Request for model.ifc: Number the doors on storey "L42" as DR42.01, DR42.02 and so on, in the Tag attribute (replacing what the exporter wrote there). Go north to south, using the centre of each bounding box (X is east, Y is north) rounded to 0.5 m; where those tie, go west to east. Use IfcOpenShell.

First a look at what the model holds.

```python
import ifcopenshell
import ifcopenshell.util.element
import ifcopenshell.util.placement

model = ifcopenshell.open("model.ifc")
print(model.schema)
storey = next(s for s in model.by_type("IfcBuildingStorey") if s.Name == "L42")
doors = [e for e in ifcopenshell.util.element.get_decomposition(storey) if e.is_a("IfcDoor")]
for e in sorted(doors, key=lambda e: e.id()):
    origin = ifcopenshell.util.placement.get_local_placement(e.ObjectPlacement)[:3, 3]
    print(e.id(), e.Tag, e.Name, origin.round(2) + 0.0, sep=" | ")
```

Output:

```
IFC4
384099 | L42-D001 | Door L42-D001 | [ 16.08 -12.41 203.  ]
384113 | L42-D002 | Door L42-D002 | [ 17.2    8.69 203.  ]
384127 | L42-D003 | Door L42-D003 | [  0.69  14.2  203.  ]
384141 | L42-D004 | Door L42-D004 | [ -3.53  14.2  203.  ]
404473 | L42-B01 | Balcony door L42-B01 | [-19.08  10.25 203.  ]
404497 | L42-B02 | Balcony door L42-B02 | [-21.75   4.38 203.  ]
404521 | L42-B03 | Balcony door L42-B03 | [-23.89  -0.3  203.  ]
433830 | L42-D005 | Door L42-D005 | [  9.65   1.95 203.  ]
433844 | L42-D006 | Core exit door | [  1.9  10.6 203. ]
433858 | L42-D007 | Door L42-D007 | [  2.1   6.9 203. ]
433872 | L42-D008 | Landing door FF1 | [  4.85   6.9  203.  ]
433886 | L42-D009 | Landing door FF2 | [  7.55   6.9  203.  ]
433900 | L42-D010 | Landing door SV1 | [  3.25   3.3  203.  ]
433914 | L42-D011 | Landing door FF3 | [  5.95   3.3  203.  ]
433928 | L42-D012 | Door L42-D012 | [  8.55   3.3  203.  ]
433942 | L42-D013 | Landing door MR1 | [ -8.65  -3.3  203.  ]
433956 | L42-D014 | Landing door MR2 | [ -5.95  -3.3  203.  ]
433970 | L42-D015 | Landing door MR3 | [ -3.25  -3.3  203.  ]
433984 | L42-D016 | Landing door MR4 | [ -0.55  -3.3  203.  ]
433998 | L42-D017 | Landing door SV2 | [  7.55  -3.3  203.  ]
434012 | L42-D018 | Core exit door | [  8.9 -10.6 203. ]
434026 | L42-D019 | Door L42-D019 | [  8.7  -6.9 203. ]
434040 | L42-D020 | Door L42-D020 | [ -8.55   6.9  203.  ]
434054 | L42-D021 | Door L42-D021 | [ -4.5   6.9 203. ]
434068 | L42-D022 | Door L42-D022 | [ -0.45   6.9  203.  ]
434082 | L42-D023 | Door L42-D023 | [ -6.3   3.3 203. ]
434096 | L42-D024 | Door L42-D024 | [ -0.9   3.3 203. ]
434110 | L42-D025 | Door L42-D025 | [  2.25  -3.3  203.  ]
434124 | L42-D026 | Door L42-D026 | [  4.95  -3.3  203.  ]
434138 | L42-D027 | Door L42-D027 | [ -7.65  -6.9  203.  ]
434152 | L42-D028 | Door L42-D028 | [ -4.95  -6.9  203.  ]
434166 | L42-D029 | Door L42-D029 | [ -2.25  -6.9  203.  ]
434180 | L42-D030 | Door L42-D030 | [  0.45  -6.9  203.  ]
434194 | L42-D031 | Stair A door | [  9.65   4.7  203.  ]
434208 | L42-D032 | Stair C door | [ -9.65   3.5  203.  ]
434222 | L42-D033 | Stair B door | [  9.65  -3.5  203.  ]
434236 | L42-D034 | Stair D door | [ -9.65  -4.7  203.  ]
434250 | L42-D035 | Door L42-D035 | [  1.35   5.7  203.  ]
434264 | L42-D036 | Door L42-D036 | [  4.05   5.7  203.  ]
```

```python
import ifcopenshell
import ifcopenshell.geom
import ifcopenshell.util.element
import ifcopenshell.util.shape

model = ifcopenshell.open("model.ifc")
settings = ifcopenshell.geom.settings()
settings.set("use-world-coords", True)


def centre(element):
    shape = ifcopenshell.geom.create_shape(settings, element)
    return ifcopenshell.util.shape.get_bbox_centroid(shape.geometry)


storey = next(s for s in model.by_type("IfcBuildingStorey") if s.Name == "L42")
doors = [e for e in ifcopenshell.util.element.get_decomposition(storey) if e.is_a("IfcDoor")]

# Insertion points can sit at a corner or the storey origin, so sort by the geometry (in metres).
centres = {e: centre(e) for e in doors}
doors.sort(key=lambda e: (-round(centres[e][1] / 0.5), centres[e][0]))

for i, e in enumerate(doors, start=1):
    number = f"DR42.{i:02d}"
    e.Tag = number
    print(e.id(), number)

model.write("model_updated.ifc")
```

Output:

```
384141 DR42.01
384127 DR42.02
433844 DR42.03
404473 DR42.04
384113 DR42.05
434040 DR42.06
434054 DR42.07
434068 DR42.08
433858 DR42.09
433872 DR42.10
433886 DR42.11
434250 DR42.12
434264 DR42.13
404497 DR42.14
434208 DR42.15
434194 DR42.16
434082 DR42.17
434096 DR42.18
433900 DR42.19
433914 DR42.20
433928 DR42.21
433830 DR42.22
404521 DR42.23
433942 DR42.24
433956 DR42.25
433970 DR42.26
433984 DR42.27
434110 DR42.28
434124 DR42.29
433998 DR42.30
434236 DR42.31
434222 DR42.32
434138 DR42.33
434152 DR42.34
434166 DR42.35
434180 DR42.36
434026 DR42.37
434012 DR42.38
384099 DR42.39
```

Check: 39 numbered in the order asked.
